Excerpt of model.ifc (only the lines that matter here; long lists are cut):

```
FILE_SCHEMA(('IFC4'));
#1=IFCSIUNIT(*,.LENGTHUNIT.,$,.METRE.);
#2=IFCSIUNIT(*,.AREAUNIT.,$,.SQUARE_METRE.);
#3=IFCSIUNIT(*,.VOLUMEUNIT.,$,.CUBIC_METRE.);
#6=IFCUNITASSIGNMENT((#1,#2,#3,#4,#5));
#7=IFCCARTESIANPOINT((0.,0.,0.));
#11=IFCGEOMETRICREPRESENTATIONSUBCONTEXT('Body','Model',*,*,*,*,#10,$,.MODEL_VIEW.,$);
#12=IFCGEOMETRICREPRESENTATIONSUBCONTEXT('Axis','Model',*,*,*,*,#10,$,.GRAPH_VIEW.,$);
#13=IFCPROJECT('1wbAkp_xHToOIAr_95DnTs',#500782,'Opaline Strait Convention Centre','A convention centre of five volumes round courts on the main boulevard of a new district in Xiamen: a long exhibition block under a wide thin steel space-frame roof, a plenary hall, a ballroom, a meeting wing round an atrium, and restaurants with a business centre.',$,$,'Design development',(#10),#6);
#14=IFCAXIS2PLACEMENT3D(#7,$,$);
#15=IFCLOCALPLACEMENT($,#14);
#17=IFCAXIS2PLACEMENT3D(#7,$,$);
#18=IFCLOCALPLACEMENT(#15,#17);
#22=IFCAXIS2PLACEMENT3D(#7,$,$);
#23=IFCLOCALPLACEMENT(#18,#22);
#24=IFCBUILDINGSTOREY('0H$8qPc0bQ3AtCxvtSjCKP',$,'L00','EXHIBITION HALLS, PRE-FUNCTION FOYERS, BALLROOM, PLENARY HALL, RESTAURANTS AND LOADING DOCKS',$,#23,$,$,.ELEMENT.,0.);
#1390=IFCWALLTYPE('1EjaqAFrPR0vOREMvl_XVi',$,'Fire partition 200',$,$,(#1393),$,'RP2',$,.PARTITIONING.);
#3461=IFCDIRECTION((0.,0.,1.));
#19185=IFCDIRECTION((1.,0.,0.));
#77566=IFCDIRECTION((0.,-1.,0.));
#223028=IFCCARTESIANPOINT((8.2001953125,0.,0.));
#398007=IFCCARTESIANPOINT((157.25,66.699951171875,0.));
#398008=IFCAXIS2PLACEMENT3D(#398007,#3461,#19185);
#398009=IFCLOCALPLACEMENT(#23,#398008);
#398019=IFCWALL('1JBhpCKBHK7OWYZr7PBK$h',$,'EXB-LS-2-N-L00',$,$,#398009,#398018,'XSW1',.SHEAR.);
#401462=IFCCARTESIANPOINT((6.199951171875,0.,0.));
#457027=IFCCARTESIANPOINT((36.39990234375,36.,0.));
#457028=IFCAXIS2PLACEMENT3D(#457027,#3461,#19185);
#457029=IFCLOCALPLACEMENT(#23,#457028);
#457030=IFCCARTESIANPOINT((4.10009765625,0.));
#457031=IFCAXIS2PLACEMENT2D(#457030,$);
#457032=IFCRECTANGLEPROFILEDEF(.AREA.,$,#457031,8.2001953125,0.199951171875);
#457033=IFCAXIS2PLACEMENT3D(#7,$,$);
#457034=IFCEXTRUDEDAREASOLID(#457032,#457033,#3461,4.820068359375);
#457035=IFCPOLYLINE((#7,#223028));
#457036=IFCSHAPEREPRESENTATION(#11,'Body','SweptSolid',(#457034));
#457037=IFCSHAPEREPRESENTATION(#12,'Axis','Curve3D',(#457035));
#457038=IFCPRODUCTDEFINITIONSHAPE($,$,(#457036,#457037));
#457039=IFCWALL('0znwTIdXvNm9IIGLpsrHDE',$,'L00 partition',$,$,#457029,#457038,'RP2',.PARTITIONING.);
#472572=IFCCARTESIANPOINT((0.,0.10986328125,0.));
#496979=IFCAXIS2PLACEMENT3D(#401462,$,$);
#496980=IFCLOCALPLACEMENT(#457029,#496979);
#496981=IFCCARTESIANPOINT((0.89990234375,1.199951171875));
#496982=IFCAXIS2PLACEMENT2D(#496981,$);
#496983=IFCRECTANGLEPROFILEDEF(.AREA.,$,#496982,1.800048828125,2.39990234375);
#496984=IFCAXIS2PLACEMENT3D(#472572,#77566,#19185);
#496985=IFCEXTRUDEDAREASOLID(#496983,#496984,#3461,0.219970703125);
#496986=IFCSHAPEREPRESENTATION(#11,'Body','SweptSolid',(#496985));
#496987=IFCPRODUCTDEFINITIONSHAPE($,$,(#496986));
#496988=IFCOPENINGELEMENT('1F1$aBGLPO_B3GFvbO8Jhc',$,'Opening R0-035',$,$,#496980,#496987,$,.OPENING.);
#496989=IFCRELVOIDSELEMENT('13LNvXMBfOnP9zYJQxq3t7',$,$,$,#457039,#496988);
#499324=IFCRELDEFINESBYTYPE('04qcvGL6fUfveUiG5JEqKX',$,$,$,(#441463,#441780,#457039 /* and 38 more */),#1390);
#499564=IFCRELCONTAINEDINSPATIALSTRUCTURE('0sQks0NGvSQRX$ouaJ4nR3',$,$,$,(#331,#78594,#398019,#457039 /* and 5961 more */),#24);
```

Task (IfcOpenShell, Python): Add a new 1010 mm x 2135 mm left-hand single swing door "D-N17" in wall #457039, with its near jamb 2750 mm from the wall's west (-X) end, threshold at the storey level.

```python
import numpy as np
import ifcopenshell
import ifcopenshell.api.feature
import ifcopenshell.api.geometry
import ifcopenshell.api.root
import ifcopenshell.api.spatial
import ifcopenshell.geom
import ifcopenshell.util.element
import ifcopenshell.util.placement
import ifcopenshell.util.representation
import ifcopenshell.util.shape
import ifcopenshell.util.unit

model = ifcopenshell.open("model.ifc")
unit_scale = ifcopenshell.util.unit.calculate_unit_scale(model)
settings = ifcopenshell.geom.settings()


def volume(element):
    """Net volume in cubic metres, openings subtracted."""
    shape = ifcopenshell.geom.create_shape(settings, element)
    return ifcopenshell.util.shape.get_volume(shape.geometry)


wall = model.by_guid("0znwTIdXvNm9IIGLpsrHDE")
storey = ifcopenshell.util.element.get_container(wall, ifc_class="IfcBuildingStorey")
context = ifcopenshell.util.representation.get_context(model, "Model", "Body", "MODEL_VIEW")
before = volume(wall)

width, height, from_end, sill = 1.01, 2.135, 2.75, 0.0  # metres

# The wall runs along its own X axis, and the end named is its -X end.
wall_shape = ifcopenshell.geom.create_shape(settings, wall)
x, y, z = ifcopenshell.util.shape.get_vertices(wall_shape.geometry).T
start = x.min() + from_end
face, thickness = float(y.min()), float(y.max() - y.min())
wall_matrix = ifcopenshell.util.placement.get_local_placement(wall.ObjectPlacement)
level = ifcopenshell.util.placement.get_local_placement(storey.ObjectPlacement)[2, 3]


def in_wall(x, y):
    """Placement at x, y metres in the wall's axes, at sill height."""
    matrix = wall_matrix.copy()
    matrix[:, 3] = wall_matrix @ np.array([x / unit_scale, y / unit_scale, 0.0, 1.0])
    matrix[2, 3] = level + sill / unit_scale
    return matrix


# Opening: a box that overshoots both wall faces by 50 mm.
opening = ifcopenshell.api.root.create_entity(model, ifc_class="IfcOpeningElement", predefined_type="OPENING")
box = ifcopenshell.api.geometry.add_wall_representation(
    model, context=context, length=width, height=height, thickness=thickness + 0.1
)
ifcopenshell.api.geometry.assign_representation(model, product=opening, representation=box)
ifcopenshell.api.geometry.edit_object_placement(model, product=opening, matrix=in_wall(start, face - 0.05), is_si=False)
ifcopenshell.api.feature.add_feature(model, feature=opening, element=wall)

door = ifcopenshell.api.root.create_entity(model, ifc_class="IfcDoor", name="D-N17", predefined_type="DOOR")
door.OverallWidth, door.OverallHeight = width / unit_scale, height / unit_scale
door.OperationType = "SINGLE_SWING_LEFT"
body = ifcopenshell.api.geometry.add_door_representation(
    model,
    context=context,
    overall_width=door.OverallWidth,
    overall_height=door.OverallHeight,
    operation_type="SINGLE_SWING_LEFT",
    lining_properties={"LiningDepth": thickness / unit_scale, "ThresholdDepth": thickness / unit_scale},
)
ifcopenshell.api.geometry.assign_representation(model, product=door, representation=body)
ifcopenshell.api.spatial.assign_container(model, products=[door], relating_structure=storey)
ifcopenshell.api.feature.add_filling(model, opening=opening, element=door)

# The lining spans the wall, so the door starts at the wall face.
ifcopenshell.api.geometry.edit_object_placement(model, product=door, matrix=in_wall(start, face), is_si=False)

after = volume(wall)

print(f"wall volume {before:.3f} -> {after:.3f} m3")

model.write("model_edited.ifc")
```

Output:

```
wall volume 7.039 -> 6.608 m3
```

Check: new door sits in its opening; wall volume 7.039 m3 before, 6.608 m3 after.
